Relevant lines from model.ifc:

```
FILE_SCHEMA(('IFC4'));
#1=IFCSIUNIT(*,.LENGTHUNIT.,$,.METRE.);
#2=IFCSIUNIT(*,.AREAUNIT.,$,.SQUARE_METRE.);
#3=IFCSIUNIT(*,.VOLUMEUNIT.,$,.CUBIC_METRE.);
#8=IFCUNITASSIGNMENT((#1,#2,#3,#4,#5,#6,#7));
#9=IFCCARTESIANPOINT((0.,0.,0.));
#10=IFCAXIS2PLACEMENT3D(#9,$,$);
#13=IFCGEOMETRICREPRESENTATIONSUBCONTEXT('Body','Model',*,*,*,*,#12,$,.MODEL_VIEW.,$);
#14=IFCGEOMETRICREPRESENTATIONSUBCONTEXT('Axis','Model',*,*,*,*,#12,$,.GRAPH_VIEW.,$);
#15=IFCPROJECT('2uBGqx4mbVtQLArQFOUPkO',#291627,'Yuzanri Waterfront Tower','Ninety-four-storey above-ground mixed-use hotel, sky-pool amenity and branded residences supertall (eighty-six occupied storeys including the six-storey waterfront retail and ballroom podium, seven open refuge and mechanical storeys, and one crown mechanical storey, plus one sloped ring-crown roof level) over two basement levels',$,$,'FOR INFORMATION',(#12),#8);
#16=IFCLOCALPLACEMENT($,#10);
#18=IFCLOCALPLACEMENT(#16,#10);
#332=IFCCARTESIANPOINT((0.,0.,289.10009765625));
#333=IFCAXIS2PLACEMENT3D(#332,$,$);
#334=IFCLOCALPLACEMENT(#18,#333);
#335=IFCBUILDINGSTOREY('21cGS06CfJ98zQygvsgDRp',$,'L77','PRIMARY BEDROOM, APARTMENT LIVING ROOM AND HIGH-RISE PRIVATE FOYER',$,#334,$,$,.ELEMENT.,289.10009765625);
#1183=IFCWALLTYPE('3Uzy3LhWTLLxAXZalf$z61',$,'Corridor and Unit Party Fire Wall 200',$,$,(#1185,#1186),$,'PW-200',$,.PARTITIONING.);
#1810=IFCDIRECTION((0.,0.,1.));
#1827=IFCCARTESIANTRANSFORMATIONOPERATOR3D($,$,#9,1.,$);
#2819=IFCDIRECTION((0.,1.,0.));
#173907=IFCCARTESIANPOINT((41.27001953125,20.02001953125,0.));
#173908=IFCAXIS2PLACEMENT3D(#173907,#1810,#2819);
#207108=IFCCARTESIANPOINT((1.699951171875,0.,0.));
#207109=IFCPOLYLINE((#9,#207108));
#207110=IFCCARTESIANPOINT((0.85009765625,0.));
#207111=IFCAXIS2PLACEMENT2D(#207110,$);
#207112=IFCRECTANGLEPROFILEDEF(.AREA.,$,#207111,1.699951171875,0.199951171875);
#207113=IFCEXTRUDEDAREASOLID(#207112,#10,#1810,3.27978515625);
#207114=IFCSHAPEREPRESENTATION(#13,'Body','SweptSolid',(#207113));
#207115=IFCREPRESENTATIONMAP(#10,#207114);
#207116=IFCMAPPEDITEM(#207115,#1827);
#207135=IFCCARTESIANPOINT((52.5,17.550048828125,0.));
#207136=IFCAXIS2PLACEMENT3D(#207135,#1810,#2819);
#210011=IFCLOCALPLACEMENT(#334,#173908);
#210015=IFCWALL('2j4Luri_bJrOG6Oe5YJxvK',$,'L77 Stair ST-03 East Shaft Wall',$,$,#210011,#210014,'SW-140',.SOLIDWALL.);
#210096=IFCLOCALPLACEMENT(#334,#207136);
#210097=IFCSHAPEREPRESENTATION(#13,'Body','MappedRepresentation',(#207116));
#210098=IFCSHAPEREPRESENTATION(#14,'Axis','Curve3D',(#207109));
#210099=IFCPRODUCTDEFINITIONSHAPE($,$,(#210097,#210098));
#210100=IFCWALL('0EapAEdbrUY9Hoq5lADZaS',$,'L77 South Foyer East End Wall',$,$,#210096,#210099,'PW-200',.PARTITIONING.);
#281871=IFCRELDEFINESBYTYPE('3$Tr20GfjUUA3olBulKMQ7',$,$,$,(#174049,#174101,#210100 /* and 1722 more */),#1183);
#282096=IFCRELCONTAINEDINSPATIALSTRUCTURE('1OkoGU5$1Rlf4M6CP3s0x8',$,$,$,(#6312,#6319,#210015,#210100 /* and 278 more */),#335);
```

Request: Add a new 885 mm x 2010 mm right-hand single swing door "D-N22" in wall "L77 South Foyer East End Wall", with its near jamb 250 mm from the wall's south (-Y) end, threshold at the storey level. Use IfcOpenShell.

```python
import numpy as np
import ifcopenshell
import ifcopenshell.api.feature
import ifcopenshell.api.geometry
import ifcopenshell.api.root
import ifcopenshell.api.spatial
import ifcopenshell.geom
import ifcopenshell.util.element
import ifcopenshell.util.placement
import ifcopenshell.util.representation
import ifcopenshell.util.shape
import ifcopenshell.util.unit

model = ifcopenshell.open("model.ifc")
unit_scale = ifcopenshell.util.unit.calculate_unit_scale(model)
settings = ifcopenshell.geom.settings()


def volume(element):
    """Net volume in cubic metres, openings subtracted."""
    shape = ifcopenshell.geom.create_shape(settings, element)
    return ifcopenshell.util.shape.get_volume(shape.geometry)


wall = model.by_id(210100)
storey = ifcopenshell.util.element.get_container(wall, ifc_class="IfcBuildingStorey")
context = ifcopenshell.util.representation.get_context(model, "Model", "Body", "MODEL_VIEW")
before = volume(wall)

width, height, from_end, sill = 0.885, 2.01, 0.25, 0.0  # metres

# The wall runs along its own X axis, and the end named is its -X end.
wall_shape = ifcopenshell.geom.create_shape(settings, wall)
x, y, z = ifcopenshell.util.shape.get_vertices(wall_shape.geometry).T
start = x.min() + from_end
face, thickness = float(y.min()), float(y.max() - y.min())
wall_matrix = ifcopenshell.util.placement.get_local_placement(wall.ObjectPlacement)
level = ifcopenshell.util.placement.get_local_placement(storey.ObjectPlacement)[2, 3]


def in_wall(x, y):
    """Placement at x, y metres in the wall's axes, at sill height."""
    matrix = wall_matrix.copy()
    matrix[:, 3] = wall_matrix @ np.array([x / unit_scale, y / unit_scale, 0.0, 1.0])
    matrix[2, 3] = level + sill / unit_scale
    return matrix


# Opening: a box that overshoots both wall faces by 50 mm.
opening = ifcopenshell.api.root.create_entity(model, ifc_class="IfcOpeningElement", predefined_type="OPENING")
box = ifcopenshell.api.geometry.add_wall_representation(
    model, context=context, length=width, height=height, thickness=thickness + 0.1
)
ifcopenshell.api.geometry.assign_representation(model, product=opening, representation=box)
ifcopenshell.api.geometry.edit_object_placement(model, product=opening, matrix=in_wall(start, face - 0.05), is_si=False)
ifcopenshell.api.feature.add_feature(model, feature=opening, element=wall)

door = ifcopenshell.api.root.create_entity(model, ifc_class="IfcDoor", name="D-N22", predefined_type="DOOR")
door.OverallWidth, door.OverallHeight = width / unit_scale, height / unit_scale
door.OperationType = "SINGLE_SWING_RIGHT"
body = ifcopenshell.api.geometry.add_door_representation(
    model,
    context=context,
    overall_width=door.OverallWidth,
    overall_height=door.OverallHeight,
    operation_type="SINGLE_SWING_RIGHT",
    lining_properties={"LiningDepth": thickness / unit_scale, "ThresholdDepth": thickness / unit_scale},
)
ifcopenshell.api.geometry.assign_representation(model, product=door, representation=body)
ifcopenshell.api.spatial.assign_container(model, products=[door], relating_structure=storey)
ifcopenshell.api.feature.add_filling(model, opening=opening, element=door)

# The lining spans the wall, so the door starts at the wall face.
ifcopenshell.api.geometry.edit_object_placement(model, product=door, matrix=in_wall(start, face), is_si=False)

after = volume(wall)

print(f"wall volume {before:.3f} -> {after:.3f} m3")

model.write("model_edited.ifc")
```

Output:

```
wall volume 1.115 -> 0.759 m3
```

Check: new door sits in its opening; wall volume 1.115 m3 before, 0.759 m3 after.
